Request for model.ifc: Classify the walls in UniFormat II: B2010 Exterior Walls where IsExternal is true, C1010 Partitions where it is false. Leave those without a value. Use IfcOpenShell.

First a look at what the model holds.

```python
import ifcopenshell
import ifcopenshell.util.element

model = ifcopenshell.open("model.ifc")
print(model.schema)
print("classifications:", [c.Name for c in model.by_type("IfcClassification")])
values = [ifcopenshell.util.element.get_pset(e, "Pset_WallCommon", "IsExternal") for e in model.by_type("IfcWall")]
for value in (True, False, None):
    print("IsExternal", value, values.count(value))
```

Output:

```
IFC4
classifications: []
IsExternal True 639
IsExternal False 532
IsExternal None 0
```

```python
import ifcopenshell
import ifcopenshell.api.classification
import ifcopenshell.util.element

model = ifcopenshell.open("model.ifc")

system = ifcopenshell.api.classification.add_classification(model, classification="UniFormat II")

walls = model.by_type("IfcWall")
external = {e: ifcopenshell.util.element.get_pset(e, "Pset_WallCommon", "IsExternal") for e in walls}
for flag, code, name in ((True, "B2010", "Exterior Walls"), (False, "C1010", "Partitions")):
    products = [e for e in walls if external[e] is flag]
    ifcopenshell.api.classification.add_reference(
        model, products=products, classification=system, identification=code, name=name
    )
    print(code, len(products))

model.write("model_v2.ifc")
```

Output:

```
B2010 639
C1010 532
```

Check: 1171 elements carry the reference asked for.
